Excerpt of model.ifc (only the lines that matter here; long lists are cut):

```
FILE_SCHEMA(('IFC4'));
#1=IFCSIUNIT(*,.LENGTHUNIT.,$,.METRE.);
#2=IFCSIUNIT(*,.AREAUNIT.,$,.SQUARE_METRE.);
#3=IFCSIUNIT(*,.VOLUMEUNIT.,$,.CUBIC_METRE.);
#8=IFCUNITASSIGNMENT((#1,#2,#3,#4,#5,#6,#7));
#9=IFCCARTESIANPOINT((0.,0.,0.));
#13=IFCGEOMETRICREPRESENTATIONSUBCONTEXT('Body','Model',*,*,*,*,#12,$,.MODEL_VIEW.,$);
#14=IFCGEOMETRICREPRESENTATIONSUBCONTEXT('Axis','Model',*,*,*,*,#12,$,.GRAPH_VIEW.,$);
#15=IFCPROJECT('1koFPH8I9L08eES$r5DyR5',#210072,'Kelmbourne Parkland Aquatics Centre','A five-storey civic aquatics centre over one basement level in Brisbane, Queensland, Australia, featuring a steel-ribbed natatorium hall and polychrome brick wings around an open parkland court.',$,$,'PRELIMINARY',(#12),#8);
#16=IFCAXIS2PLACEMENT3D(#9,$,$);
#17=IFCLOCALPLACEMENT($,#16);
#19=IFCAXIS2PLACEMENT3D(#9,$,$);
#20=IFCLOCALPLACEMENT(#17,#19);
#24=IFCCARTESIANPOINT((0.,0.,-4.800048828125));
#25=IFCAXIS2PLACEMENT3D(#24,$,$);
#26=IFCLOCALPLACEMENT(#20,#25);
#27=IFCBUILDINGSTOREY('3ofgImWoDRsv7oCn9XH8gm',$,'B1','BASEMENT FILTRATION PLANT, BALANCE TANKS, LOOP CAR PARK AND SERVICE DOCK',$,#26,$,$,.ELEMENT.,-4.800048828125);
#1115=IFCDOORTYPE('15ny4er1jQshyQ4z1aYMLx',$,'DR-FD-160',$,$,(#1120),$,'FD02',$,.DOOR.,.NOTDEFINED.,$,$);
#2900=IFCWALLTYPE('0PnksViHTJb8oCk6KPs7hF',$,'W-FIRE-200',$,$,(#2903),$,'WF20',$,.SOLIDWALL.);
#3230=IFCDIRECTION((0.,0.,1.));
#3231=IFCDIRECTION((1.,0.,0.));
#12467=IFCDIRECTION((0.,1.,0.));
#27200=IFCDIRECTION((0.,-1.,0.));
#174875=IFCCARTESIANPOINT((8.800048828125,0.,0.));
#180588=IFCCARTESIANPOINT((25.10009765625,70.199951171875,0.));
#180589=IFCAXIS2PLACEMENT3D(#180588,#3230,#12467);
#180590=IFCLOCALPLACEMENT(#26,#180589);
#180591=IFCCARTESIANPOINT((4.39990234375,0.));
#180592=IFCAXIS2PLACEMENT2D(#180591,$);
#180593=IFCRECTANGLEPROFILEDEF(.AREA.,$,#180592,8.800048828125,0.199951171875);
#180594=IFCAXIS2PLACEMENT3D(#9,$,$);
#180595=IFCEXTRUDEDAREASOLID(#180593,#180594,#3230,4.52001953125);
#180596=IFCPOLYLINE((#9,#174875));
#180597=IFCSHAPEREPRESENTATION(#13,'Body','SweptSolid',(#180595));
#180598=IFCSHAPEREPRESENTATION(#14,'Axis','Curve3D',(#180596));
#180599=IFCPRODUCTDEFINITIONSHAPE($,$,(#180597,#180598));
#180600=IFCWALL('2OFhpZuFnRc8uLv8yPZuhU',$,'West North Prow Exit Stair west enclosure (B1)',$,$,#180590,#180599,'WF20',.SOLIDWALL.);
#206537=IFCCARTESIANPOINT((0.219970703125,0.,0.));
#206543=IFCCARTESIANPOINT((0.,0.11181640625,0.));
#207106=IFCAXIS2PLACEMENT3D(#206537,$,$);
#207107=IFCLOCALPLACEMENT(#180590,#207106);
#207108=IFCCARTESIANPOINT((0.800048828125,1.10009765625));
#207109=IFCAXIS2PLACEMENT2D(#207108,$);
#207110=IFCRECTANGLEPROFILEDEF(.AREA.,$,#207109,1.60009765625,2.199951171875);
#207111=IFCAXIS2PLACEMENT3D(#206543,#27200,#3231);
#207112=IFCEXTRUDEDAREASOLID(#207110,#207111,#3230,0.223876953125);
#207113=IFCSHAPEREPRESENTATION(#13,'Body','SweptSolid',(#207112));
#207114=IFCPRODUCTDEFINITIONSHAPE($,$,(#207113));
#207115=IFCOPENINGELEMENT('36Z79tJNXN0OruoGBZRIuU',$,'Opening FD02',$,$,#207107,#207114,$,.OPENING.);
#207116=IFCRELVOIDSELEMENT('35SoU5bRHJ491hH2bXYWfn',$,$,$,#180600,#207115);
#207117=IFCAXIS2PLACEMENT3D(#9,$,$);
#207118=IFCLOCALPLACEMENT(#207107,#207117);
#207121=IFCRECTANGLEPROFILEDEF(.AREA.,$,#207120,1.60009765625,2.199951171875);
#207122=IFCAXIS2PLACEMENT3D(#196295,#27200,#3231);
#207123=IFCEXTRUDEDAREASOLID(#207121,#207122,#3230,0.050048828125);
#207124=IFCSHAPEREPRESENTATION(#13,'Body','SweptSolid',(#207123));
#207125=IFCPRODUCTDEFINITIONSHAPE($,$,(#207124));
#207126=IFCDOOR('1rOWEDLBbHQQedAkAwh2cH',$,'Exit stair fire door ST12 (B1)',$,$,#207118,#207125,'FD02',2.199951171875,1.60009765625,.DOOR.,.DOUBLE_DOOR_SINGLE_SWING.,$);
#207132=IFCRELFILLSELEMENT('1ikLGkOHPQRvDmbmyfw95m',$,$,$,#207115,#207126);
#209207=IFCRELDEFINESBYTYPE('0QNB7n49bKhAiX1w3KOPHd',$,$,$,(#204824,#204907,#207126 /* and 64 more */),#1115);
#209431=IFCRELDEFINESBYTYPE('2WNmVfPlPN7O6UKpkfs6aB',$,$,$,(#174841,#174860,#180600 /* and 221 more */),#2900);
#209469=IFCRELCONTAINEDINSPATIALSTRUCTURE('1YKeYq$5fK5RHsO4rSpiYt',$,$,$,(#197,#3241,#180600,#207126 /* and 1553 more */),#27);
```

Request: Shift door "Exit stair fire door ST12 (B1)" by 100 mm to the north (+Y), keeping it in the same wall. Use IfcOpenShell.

```python
import ifcopenshell
import ifcopenshell.api.geometry
import ifcopenshell.util.placement
import ifcopenshell.util.unit

model = ifcopenshell.open("model.ifc")
unit_scale = ifcopenshell.util.unit.calculate_unit_scale(model)

door = model.by_id(207126)
opening = door.FillsVoids[0].RelatingOpeningElement
wall = opening.VoidsElements[0].RelatingBuildingElement

wall_matrix = ifcopenshell.util.placement.get_local_placement(wall.ObjectPlacement)
shift = wall_matrix[:3, 0] * 0.1 / unit_scale
before = ifcopenshell.util.placement.get_local_placement(door.ObjectPlacement)[:3, 3].copy()

# The door is placed relative to its opening, so it follows when the opening moves.
matrix = ifcopenshell.util.placement.get_local_placement(opening.ObjectPlacement)
matrix[:3, 3] += shift
ifcopenshell.api.geometry.edit_object_placement(
    model, product=opening, matrix=matrix, is_si=False, should_transform_children=True
)

after = ifcopenshell.util.placement.get_local_placement(door.ObjectPlacement)[:3, 3]
print("door moved by", (after - before).round(3) + 0.0)

model.write("model_rev.ifc")
```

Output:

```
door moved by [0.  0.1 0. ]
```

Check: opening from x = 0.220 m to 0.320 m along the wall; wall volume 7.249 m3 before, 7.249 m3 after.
